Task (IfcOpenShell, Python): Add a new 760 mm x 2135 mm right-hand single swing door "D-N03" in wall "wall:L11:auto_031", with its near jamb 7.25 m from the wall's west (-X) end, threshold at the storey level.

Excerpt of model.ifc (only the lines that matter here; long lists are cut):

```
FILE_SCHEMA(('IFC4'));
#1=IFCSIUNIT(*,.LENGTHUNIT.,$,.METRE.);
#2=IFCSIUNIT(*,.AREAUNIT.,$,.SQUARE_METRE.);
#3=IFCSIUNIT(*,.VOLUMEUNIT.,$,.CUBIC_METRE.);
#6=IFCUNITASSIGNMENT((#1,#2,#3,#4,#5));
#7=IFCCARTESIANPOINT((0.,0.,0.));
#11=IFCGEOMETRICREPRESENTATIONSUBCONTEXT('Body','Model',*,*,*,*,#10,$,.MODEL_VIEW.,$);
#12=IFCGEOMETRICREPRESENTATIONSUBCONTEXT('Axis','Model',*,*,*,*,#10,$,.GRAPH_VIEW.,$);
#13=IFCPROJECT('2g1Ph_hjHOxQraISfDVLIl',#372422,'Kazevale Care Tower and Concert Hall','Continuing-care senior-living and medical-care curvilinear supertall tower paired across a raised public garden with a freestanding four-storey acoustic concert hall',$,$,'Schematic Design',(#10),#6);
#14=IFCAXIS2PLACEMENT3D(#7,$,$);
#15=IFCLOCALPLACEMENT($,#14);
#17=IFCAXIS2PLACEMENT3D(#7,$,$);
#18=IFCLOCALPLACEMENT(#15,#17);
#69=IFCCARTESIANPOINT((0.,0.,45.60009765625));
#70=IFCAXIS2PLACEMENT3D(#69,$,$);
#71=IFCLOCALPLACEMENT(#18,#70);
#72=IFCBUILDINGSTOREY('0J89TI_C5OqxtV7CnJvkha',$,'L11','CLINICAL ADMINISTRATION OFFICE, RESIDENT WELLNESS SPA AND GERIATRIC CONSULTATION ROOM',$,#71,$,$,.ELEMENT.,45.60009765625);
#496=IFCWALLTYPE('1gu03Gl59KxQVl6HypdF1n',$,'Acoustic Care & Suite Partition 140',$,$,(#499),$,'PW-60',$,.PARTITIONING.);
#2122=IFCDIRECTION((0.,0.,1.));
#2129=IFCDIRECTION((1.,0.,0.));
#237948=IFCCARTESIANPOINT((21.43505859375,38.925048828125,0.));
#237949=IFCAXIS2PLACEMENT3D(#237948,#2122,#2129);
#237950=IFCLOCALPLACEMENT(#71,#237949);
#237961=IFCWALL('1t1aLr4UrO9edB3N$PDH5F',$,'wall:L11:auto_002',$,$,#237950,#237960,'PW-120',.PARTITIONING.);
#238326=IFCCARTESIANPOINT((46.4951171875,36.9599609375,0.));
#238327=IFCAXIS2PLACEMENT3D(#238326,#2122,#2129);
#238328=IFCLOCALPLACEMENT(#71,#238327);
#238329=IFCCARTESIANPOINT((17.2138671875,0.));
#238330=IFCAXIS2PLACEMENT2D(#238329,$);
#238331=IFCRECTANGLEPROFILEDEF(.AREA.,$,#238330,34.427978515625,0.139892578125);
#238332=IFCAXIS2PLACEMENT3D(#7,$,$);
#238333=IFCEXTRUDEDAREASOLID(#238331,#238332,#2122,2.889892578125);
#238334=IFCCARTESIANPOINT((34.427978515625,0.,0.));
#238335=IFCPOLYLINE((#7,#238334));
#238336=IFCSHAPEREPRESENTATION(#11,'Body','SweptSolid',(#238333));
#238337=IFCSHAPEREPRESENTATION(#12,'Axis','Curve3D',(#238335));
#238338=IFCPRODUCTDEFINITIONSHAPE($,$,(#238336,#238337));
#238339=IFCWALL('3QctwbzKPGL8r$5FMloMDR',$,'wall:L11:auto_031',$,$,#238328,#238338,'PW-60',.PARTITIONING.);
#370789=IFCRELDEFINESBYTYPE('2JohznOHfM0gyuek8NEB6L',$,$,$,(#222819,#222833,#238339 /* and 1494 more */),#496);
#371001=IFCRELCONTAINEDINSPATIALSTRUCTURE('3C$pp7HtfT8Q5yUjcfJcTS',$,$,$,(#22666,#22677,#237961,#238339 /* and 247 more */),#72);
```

```python
import numpy as np
import ifcopenshell
import ifcopenshell.api.feature
import ifcopenshell.api.geometry
import ifcopenshell.api.root
import ifcopenshell.api.spatial
import ifcopenshell.geom
import ifcopenshell.util.element
import ifcopenshell.util.placement
import ifcopenshell.util.representation
import ifcopenshell.util.shape
import ifcopenshell.util.unit

model = ifcopenshell.open("model.ifc")
unit_scale = ifcopenshell.util.unit.calculate_unit_scale(model)
settings = ifcopenshell.geom.settings()


def volume(element):
    """Net volume in cubic metres, openings subtracted."""
    shape = ifcopenshell.geom.create_shape(settings, element)
    return ifcopenshell.util.shape.get_volume(shape.geometry)


wall = model.by_id(238339)
storey = ifcopenshell.util.element.get_container(wall, ifc_class="IfcBuildingStorey")
context = ifcopenshell.util.representation.get_context(model, "Model", "Body", "MODEL_VIEW")
before = volume(wall)

width, height, from_end, sill = 0.76, 2.135, 7.25, 0.0  # metres

# The wall runs along its own X axis, and the end named is its -X end.
wall_shape = ifcopenshell.geom.create_shape(settings, wall)
x, y, z = ifcopenshell.util.shape.get_vertices(wall_shape.geometry).T
start = x.min() + from_end
face, thickness = float(y.min()), float(y.max() - y.min())
wall_matrix = ifcopenshell.util.placement.get_local_placement(wall.ObjectPlacement)
level = ifcopenshell.util.placement.get_local_placement(storey.ObjectPlacement)[2, 3]


def in_wall(x, y):
    """Placement at x, y metres in the wall's axes, at sill height."""
    matrix = wall_matrix.copy()
    matrix[:, 3] = wall_matrix @ np.array([x / unit_scale, y / unit_scale, 0.0, 1.0])
    matrix[2, 3] = level + sill / unit_scale
    return matrix


# Opening: a box that overshoots both wall faces by 50 mm.
opening = ifcopenshell.api.root.create_entity(model, ifc_class="IfcOpeningElement", predefined_type="OPENING")
box = ifcopenshell.api.geometry.add_wall_representation(
    model, context=context, length=width, height=height, thickness=thickness + 0.1
)
ifcopenshell.api.geometry.assign_representation(model, product=opening, representation=box)
ifcopenshell.api.geometry.edit_object_placement(model, product=opening, matrix=in_wall(start, face - 0.05), is_si=False)
ifcopenshell.api.feature.add_feature(model, feature=opening, element=wall)

door = ifcopenshell.api.root.create_entity(model, ifc_class="IfcDoor", name="D-N03", predefined_type="DOOR")
door.OverallWidth, door.OverallHeight = width / unit_scale, height / unit_scale
door.OperationType = "SINGLE_SWING_RIGHT"
body = ifcopenshell.api.geometry.add_door_representation(
    model,
    context=context,
    overall_width=door.OverallWidth,
    overall_height=door.OverallHeight,
    operation_type="SINGLE_SWING_RIGHT",
    lining_properties={"LiningDepth": thickness / unit_scale, "ThresholdDepth": thickness / unit_scale},
)
ifcopenshell.api.geometry.assign_representation(model, product=door, representation=body)
ifcopenshell.api.spatial.assign_container(model, products=[door], relating_structure=storey)
ifcopenshell.api.feature.add_filling(model, opening=opening, element=door)

# The lining spans the wall, so the door starts at the wall face.
ifcopenshell.api.geometry.edit_object_placement(model, product=door, matrix=in_wall(start, face), is_si=False)

after = volume(wall)

print(f"wall volume {before:.3f} -> {after:.3f} m3")

model.write("model_v2.ifc")
```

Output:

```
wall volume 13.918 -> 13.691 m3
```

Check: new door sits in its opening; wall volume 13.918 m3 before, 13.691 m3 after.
